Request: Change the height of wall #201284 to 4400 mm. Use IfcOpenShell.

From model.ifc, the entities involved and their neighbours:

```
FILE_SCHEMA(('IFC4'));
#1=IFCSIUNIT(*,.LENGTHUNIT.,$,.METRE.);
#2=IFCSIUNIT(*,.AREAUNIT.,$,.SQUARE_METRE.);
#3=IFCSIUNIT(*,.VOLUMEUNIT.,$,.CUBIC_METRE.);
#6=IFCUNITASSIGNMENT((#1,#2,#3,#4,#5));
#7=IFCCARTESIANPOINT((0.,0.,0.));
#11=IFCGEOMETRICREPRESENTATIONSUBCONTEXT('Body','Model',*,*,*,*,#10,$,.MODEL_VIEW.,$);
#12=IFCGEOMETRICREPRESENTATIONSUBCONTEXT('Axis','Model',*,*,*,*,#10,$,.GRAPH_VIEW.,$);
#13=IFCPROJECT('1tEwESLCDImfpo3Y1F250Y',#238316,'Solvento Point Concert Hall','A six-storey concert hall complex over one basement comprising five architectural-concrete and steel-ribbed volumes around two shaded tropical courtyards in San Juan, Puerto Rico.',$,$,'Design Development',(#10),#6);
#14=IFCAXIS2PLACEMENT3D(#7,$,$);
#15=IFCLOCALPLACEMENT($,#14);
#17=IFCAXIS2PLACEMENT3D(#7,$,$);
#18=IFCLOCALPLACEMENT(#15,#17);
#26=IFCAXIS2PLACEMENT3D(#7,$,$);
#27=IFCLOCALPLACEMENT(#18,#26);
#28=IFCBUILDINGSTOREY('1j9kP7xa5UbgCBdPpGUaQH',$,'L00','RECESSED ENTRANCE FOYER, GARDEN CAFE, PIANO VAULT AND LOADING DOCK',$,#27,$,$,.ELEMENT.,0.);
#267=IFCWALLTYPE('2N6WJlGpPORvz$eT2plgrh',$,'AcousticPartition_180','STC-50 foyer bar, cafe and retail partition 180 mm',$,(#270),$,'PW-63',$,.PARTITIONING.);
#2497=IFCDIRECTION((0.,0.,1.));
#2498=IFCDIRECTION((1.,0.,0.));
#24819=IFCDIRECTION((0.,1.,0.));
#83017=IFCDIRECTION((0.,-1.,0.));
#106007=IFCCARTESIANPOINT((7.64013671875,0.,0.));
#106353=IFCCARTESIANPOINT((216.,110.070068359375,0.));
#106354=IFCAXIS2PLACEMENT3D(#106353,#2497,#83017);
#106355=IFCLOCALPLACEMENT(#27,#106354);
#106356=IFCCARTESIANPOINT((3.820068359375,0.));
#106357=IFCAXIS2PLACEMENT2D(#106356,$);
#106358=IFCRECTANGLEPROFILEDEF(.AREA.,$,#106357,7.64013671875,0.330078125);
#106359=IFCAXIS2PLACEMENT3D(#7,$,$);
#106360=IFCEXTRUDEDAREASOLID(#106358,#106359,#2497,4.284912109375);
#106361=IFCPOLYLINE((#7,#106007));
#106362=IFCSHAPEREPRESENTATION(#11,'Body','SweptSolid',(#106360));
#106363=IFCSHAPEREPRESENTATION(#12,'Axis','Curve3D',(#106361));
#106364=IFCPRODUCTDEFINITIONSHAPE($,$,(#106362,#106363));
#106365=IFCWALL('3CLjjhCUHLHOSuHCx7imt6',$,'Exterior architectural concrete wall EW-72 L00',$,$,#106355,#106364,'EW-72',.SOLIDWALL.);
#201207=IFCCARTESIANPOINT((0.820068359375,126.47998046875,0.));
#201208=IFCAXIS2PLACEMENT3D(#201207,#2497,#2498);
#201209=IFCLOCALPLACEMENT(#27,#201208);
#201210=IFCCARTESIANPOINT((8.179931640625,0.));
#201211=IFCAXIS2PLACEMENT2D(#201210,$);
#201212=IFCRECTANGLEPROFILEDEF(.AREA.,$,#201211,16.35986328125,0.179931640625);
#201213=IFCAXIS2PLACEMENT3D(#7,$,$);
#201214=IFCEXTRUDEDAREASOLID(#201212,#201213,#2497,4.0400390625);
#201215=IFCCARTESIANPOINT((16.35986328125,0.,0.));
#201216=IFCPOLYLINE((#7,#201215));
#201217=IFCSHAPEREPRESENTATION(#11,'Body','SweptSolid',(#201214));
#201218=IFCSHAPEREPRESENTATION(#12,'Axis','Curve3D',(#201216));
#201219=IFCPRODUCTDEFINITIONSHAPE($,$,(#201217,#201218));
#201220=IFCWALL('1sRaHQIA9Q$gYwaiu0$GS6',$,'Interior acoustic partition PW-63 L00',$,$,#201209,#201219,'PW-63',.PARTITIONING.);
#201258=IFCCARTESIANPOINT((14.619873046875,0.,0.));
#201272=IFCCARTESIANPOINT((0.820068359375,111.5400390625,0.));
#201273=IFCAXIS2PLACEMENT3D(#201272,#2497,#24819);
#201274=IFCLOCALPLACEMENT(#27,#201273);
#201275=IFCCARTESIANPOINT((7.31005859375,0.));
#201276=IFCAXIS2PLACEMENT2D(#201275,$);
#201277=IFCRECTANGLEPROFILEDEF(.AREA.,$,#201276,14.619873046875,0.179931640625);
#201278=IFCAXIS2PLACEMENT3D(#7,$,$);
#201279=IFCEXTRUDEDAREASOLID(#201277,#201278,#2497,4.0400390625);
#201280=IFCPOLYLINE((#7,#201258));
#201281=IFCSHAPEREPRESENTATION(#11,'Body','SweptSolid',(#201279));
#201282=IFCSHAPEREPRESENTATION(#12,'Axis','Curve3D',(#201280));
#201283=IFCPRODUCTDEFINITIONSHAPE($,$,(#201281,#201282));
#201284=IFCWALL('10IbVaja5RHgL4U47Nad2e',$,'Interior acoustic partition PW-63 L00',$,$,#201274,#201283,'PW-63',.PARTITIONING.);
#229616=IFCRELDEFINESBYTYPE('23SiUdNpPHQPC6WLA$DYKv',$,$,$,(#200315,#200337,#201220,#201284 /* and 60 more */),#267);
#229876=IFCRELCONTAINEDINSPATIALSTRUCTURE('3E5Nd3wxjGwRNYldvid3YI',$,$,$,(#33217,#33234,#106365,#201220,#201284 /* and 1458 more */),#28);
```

```python
import ifcopenshell
import ifcopenshell.geom
import ifcopenshell.util.representation
import ifcopenshell.util.shape
import ifcopenshell.util.unit

model = ifcopenshell.open("model.ifc")
unit_scale = ifcopenshell.util.unit.calculate_unit_scale(model)
settings = ifcopenshell.geom.settings()


def volume(element):
    """Net volume in cubic metres, openings subtracted."""
    shape = ifcopenshell.geom.create_shape(settings, element)
    return ifcopenshell.util.shape.get_volume(shape.geometry)


wall = model.by_guid("10IbVaja5RHgL4U47Nad2e")
before = volume(wall)

body = ifcopenshell.util.representation.get_representation(wall, "Model", "Body")
solid = body.Items[0]
old_height = solid.Depth
solid.Depth = 4.4 / unit_scale
after = volume(wall)

print(f"height {old_height:g} -> {solid.Depth:g}, volume {before:.3f} -> {after:.3f} m3")

model.write("model_v2.ifc")
```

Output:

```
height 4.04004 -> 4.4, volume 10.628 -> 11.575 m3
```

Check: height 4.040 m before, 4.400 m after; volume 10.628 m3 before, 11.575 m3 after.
